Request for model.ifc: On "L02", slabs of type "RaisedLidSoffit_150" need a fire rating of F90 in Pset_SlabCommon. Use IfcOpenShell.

First a look at what the model holds.

```python
import ifcopenshell
import ifcopenshell.util.element

model = ifcopenshell.open("model.ifc")
print(model.schema)
storey = next(s for s in model.by_type("IfcBuildingStorey") if s.Name == "L02")
slabs = [e for e in ifcopenshell.util.element.get_decomposition(storey) if e.is_a("IfcSlab")]
seen = {}
for e in slabs:
    element_type = ifcopenshell.util.element.get_type(e)
    key = (element_type.Name if element_type != e and element_type else None, ifcopenshell.util.element.get_pset(e, "Pset_SlabCommon", "FireRating"))
    seen[key] = seen.get(key, 0) + 1
for (name, value), count in sorted(seen.items(), key=str):
    print(count, "x", name, "|", value)
```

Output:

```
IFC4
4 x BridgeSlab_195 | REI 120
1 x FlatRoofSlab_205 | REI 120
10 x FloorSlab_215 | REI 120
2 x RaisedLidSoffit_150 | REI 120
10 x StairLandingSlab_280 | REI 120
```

```python
import ifcopenshell
import ifcopenshell.api.pset
import ifcopenshell.util.element

model = ifcopenshell.open("model.ifc")

storey = next(s for s in model.by_type("IfcBuildingStorey") if s.Name == "L02")
slabs = [e for e in ifcopenshell.util.element.get_decomposition(storey) if e.is_a("IfcSlab")]

count = 0
for e in slabs:
    element_type = ifcopenshell.util.element.get_type(e)
    if element_type in (None, e) or element_type.Name != "RaisedLidSoffit_150":
        continue
    # add_pset returns the element's existing set when there is one.
    pset = ifcopenshell.api.pset.add_pset(model, product=e, name="Pset_SlabCommon")
    ifcopenshell.api.pset.edit_pset(model, pset=pset, properties={"FireRating": "F90"})
    count += 1

print(count, "slabs updated")

model.write("model_updated.ifc")
```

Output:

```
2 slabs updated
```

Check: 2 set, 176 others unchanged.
